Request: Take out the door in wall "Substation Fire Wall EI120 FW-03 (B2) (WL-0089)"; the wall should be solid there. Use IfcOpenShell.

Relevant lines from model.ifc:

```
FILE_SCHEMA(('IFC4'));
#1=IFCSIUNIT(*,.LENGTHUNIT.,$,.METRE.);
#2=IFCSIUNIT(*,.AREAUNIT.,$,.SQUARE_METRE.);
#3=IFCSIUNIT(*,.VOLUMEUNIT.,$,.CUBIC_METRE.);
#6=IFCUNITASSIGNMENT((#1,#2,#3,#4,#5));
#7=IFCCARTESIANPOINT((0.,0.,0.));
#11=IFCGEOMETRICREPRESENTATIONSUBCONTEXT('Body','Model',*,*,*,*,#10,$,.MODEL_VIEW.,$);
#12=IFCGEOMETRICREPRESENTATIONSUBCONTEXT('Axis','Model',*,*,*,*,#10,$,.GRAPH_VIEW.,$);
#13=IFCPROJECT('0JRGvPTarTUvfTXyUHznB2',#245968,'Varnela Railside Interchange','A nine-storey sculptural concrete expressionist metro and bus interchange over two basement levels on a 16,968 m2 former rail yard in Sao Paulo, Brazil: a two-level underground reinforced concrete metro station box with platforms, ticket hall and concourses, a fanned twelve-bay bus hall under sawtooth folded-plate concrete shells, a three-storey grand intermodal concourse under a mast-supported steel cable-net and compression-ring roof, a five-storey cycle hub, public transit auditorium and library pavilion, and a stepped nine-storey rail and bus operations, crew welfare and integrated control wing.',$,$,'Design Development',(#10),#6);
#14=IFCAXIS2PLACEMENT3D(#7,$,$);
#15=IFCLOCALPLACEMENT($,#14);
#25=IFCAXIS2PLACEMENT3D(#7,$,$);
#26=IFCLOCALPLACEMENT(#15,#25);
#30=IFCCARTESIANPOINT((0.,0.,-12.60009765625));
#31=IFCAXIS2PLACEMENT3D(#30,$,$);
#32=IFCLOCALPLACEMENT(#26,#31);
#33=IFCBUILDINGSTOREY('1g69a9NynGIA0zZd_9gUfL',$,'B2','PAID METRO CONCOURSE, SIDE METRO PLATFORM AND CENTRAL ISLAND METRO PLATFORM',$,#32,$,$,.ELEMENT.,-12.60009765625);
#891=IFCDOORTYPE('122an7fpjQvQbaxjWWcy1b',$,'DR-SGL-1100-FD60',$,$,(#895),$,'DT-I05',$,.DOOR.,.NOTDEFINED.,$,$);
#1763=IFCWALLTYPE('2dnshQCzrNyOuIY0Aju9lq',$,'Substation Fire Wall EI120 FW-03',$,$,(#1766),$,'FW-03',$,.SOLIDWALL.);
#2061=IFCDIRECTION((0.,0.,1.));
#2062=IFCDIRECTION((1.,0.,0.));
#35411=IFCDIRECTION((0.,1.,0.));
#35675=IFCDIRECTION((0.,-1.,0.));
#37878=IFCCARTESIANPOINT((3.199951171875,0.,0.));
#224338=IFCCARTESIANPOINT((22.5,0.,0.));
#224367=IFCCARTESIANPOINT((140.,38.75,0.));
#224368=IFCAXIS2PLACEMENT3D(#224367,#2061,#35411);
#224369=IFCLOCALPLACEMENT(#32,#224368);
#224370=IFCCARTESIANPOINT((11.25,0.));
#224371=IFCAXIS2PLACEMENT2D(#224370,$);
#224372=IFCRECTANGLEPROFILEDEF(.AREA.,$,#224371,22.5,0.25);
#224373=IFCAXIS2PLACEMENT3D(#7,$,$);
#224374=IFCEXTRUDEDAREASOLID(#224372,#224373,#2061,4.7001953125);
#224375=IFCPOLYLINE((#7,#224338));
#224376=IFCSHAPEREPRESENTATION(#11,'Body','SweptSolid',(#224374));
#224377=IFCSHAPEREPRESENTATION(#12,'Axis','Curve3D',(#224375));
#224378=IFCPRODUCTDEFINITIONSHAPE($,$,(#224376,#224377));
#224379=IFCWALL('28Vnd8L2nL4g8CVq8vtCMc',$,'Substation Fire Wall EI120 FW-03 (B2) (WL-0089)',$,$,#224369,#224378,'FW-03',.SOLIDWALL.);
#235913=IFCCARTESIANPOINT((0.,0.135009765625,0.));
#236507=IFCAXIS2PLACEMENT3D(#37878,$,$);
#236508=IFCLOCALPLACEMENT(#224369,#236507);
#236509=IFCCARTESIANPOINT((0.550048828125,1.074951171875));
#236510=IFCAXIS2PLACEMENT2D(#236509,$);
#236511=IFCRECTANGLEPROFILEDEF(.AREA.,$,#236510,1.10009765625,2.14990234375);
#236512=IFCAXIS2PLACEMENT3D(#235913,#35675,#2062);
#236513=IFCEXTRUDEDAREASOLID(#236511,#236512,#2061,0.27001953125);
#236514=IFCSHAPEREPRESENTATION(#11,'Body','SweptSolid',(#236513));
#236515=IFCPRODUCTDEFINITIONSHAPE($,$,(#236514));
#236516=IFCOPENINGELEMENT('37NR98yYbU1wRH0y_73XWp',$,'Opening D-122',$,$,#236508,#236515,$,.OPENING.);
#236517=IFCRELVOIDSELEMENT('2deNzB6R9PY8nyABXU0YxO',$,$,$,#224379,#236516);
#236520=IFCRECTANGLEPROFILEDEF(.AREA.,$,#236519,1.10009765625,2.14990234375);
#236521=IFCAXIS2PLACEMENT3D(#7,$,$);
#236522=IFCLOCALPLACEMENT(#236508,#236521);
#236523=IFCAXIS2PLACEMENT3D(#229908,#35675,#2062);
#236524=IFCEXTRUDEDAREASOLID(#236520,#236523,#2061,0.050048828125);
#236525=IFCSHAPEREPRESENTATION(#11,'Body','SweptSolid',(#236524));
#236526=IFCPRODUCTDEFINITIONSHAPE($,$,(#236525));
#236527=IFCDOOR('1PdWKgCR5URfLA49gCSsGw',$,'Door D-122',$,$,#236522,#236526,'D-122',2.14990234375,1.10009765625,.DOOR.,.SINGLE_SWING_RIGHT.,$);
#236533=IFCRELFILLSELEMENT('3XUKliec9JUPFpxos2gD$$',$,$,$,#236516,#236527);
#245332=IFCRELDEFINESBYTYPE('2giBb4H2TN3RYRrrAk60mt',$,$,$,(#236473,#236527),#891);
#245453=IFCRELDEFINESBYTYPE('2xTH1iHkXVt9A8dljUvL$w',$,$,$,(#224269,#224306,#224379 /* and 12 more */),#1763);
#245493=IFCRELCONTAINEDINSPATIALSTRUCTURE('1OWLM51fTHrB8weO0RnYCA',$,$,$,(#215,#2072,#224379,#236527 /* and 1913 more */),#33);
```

```python
import ifcopenshell
import ifcopenshell.api.feature
import ifcopenshell.api.root
import ifcopenshell.geom
import ifcopenshell.util.shape

model = ifcopenshell.open("model.ifc")
settings = ifcopenshell.geom.settings()


def volume(element):
    """Net volume in cubic metres, openings subtracted."""
    shape = ifcopenshell.geom.create_shape(settings, element)
    return ifcopenshell.util.shape.get_volume(shape.geometry)


door = model.by_id(236527)
opening = door.FillsVoids[0].RelatingOpeningElement
wall = opening.VoidsElements[0].RelatingBuildingElement
before = volume(wall)

ifcopenshell.api.root.remove_product(model, product=door)
ifcopenshell.api.feature.remove_feature(model, feature=opening)

after = volume(wall)

print(f"wall volume {before:.3f} -> {after:.3f} m3")

model.write("model_updated.ifc")
```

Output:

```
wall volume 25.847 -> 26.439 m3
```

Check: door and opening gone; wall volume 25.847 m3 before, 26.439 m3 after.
